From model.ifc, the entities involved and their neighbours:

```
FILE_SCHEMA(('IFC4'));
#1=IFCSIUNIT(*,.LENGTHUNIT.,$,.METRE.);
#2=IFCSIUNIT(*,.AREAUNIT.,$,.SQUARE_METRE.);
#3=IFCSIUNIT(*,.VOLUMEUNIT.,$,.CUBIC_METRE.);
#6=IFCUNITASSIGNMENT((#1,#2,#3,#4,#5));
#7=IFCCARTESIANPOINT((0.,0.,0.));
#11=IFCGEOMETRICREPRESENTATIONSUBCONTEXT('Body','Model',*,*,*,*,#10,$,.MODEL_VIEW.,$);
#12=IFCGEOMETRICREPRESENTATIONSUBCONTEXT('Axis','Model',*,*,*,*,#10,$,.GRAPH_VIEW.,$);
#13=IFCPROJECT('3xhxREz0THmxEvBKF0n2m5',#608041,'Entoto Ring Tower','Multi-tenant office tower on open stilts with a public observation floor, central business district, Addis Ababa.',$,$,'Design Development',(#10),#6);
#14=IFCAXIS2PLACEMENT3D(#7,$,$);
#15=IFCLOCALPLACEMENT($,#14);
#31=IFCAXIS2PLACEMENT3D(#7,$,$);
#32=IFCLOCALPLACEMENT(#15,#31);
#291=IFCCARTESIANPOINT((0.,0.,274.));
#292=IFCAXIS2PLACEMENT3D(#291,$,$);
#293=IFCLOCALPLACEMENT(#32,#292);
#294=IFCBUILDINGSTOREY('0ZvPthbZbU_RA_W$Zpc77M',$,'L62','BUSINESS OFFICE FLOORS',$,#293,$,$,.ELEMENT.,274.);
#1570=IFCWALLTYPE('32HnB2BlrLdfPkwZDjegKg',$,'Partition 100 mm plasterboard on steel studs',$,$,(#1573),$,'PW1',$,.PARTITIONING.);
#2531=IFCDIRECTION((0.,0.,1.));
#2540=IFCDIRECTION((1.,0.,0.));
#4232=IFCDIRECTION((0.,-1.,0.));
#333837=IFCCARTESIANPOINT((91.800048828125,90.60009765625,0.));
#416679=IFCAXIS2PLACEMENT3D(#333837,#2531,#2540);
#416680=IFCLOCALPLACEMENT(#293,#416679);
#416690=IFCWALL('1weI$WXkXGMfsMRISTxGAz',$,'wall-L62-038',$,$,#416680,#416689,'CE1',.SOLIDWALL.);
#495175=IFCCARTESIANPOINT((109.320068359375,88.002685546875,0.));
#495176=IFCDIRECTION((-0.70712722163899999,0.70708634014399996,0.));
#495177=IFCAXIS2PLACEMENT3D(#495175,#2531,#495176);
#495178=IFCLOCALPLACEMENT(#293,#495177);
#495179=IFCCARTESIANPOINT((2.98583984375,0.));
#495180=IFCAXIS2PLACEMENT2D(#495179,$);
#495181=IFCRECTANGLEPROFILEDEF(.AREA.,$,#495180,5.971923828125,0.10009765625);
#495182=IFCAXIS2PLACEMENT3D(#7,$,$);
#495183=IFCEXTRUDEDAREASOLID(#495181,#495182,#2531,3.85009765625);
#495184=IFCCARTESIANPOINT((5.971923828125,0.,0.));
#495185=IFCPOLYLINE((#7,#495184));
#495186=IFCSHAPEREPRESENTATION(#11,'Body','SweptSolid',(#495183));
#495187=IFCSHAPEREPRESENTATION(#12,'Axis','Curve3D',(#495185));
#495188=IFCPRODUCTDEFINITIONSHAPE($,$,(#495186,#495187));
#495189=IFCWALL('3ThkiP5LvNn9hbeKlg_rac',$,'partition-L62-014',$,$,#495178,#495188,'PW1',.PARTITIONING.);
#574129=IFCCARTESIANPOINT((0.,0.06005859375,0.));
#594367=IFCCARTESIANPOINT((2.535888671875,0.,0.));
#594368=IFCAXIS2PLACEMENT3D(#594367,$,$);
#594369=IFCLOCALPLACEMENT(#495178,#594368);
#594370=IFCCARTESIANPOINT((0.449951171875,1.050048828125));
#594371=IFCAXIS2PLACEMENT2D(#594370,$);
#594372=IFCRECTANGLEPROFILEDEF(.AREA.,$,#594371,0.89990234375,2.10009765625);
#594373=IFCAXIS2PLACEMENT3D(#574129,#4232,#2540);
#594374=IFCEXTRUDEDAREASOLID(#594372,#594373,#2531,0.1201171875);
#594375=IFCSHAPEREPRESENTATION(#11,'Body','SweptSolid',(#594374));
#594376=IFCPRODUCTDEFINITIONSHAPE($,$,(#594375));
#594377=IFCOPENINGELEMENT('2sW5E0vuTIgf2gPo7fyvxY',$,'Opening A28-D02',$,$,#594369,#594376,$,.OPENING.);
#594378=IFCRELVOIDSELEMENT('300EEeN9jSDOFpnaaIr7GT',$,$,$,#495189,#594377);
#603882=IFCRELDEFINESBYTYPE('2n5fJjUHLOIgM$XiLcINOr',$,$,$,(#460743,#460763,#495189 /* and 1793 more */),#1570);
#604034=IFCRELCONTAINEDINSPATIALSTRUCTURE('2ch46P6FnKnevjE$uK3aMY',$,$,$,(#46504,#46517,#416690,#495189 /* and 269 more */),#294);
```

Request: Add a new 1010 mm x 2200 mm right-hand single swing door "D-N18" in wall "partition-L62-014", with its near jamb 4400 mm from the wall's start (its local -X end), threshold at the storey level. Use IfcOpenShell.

```python
import numpy as np
import ifcopenshell
import ifcopenshell.api.feature
import ifcopenshell.api.geometry
import ifcopenshell.api.root
import ifcopenshell.api.spatial
import ifcopenshell.geom
import ifcopenshell.util.element
import ifcopenshell.util.placement
import ifcopenshell.util.representation
import ifcopenshell.util.shape
import ifcopenshell.util.unit

model = ifcopenshell.open("model.ifc")
unit_scale = ifcopenshell.util.unit.calculate_unit_scale(model)
settings = ifcopenshell.geom.settings()


def volume(element):
    """Net volume in cubic metres, openings subtracted."""
    shape = ifcopenshell.geom.create_shape(settings, element)
    return ifcopenshell.util.shape.get_volume(shape.geometry)


wall = model.by_guid("3ThkiP5LvNn9hbeKlg_rac")
storey = ifcopenshell.util.element.get_container(wall, ifc_class="IfcBuildingStorey")
context = ifcopenshell.util.representation.get_context(model, "Model", "Body", "MODEL_VIEW")
before = volume(wall)

width, height, from_end, sill = 1.01, 2.2, 4.4, 0.0  # metres

# The wall runs along its own X axis, and the end named is its -X end.
wall_shape = ifcopenshell.geom.create_shape(settings, wall)
x, y, z = ifcopenshell.util.shape.get_vertices(wall_shape.geometry).T
start = x.min() + from_end
face, thickness = float(y.min()), float(y.max() - y.min())
wall_matrix = ifcopenshell.util.placement.get_local_placement(wall.ObjectPlacement)
level = ifcopenshell.util.placement.get_local_placement(storey.ObjectPlacement)[2, 3]


def in_wall(x, y):
    """Placement at x, y metres in the wall's axes, at sill height."""
    matrix = wall_matrix.copy()
    matrix[:, 3] = wall_matrix @ np.array([x / unit_scale, y / unit_scale, 0.0, 1.0])
    matrix[2, 3] = level + sill / unit_scale
    return matrix


# Opening: a box that overshoots both wall faces by 50 mm.
opening = ifcopenshell.api.root.create_entity(model, ifc_class="IfcOpeningElement", predefined_type="OPENING")
box = ifcopenshell.api.geometry.add_wall_representation(
    model, context=context, length=width, height=height, thickness=thickness + 0.1
)
ifcopenshell.api.geometry.assign_representation(model, product=opening, representation=box)
ifcopenshell.api.geometry.edit_object_placement(model, product=opening, matrix=in_wall(start, face - 0.05), is_si=False)
ifcopenshell.api.feature.add_feature(model, feature=opening, element=wall)

door = ifcopenshell.api.root.create_entity(model, ifc_class="IfcDoor", name="D-N18", predefined_type="DOOR")
door.OverallWidth, door.OverallHeight = width / unit_scale, height / unit_scale
door.OperationType = "SINGLE_SWING_RIGHT"
body = ifcopenshell.api.geometry.add_door_representation(
    model,
    context=context,
    overall_width=door.OverallWidth,
    overall_height=door.OverallHeight,
    operation_type="SINGLE_SWING_RIGHT",
    lining_properties={"LiningDepth": thickness / unit_scale, "ThresholdDepth": thickness / unit_scale},
)
ifcopenshell.api.geometry.assign_representation(model, product=door, representation=body)
ifcopenshell.api.spatial.assign_container(model, products=[door], relating_structure=storey)
ifcopenshell.api.feature.add_filling(model, opening=opening, element=door)

# The lining spans the wall, so the door starts at the wall face.
ifcopenshell.api.geometry.edit_object_placement(model, product=door, matrix=in_wall(start, face), is_si=False)

after = volume(wall)

print(f"wall volume {before:.3f} -> {after:.3f} m3")

model.write("model_updated.ifc")
```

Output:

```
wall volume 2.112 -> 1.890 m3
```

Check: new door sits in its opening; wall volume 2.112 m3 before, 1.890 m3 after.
